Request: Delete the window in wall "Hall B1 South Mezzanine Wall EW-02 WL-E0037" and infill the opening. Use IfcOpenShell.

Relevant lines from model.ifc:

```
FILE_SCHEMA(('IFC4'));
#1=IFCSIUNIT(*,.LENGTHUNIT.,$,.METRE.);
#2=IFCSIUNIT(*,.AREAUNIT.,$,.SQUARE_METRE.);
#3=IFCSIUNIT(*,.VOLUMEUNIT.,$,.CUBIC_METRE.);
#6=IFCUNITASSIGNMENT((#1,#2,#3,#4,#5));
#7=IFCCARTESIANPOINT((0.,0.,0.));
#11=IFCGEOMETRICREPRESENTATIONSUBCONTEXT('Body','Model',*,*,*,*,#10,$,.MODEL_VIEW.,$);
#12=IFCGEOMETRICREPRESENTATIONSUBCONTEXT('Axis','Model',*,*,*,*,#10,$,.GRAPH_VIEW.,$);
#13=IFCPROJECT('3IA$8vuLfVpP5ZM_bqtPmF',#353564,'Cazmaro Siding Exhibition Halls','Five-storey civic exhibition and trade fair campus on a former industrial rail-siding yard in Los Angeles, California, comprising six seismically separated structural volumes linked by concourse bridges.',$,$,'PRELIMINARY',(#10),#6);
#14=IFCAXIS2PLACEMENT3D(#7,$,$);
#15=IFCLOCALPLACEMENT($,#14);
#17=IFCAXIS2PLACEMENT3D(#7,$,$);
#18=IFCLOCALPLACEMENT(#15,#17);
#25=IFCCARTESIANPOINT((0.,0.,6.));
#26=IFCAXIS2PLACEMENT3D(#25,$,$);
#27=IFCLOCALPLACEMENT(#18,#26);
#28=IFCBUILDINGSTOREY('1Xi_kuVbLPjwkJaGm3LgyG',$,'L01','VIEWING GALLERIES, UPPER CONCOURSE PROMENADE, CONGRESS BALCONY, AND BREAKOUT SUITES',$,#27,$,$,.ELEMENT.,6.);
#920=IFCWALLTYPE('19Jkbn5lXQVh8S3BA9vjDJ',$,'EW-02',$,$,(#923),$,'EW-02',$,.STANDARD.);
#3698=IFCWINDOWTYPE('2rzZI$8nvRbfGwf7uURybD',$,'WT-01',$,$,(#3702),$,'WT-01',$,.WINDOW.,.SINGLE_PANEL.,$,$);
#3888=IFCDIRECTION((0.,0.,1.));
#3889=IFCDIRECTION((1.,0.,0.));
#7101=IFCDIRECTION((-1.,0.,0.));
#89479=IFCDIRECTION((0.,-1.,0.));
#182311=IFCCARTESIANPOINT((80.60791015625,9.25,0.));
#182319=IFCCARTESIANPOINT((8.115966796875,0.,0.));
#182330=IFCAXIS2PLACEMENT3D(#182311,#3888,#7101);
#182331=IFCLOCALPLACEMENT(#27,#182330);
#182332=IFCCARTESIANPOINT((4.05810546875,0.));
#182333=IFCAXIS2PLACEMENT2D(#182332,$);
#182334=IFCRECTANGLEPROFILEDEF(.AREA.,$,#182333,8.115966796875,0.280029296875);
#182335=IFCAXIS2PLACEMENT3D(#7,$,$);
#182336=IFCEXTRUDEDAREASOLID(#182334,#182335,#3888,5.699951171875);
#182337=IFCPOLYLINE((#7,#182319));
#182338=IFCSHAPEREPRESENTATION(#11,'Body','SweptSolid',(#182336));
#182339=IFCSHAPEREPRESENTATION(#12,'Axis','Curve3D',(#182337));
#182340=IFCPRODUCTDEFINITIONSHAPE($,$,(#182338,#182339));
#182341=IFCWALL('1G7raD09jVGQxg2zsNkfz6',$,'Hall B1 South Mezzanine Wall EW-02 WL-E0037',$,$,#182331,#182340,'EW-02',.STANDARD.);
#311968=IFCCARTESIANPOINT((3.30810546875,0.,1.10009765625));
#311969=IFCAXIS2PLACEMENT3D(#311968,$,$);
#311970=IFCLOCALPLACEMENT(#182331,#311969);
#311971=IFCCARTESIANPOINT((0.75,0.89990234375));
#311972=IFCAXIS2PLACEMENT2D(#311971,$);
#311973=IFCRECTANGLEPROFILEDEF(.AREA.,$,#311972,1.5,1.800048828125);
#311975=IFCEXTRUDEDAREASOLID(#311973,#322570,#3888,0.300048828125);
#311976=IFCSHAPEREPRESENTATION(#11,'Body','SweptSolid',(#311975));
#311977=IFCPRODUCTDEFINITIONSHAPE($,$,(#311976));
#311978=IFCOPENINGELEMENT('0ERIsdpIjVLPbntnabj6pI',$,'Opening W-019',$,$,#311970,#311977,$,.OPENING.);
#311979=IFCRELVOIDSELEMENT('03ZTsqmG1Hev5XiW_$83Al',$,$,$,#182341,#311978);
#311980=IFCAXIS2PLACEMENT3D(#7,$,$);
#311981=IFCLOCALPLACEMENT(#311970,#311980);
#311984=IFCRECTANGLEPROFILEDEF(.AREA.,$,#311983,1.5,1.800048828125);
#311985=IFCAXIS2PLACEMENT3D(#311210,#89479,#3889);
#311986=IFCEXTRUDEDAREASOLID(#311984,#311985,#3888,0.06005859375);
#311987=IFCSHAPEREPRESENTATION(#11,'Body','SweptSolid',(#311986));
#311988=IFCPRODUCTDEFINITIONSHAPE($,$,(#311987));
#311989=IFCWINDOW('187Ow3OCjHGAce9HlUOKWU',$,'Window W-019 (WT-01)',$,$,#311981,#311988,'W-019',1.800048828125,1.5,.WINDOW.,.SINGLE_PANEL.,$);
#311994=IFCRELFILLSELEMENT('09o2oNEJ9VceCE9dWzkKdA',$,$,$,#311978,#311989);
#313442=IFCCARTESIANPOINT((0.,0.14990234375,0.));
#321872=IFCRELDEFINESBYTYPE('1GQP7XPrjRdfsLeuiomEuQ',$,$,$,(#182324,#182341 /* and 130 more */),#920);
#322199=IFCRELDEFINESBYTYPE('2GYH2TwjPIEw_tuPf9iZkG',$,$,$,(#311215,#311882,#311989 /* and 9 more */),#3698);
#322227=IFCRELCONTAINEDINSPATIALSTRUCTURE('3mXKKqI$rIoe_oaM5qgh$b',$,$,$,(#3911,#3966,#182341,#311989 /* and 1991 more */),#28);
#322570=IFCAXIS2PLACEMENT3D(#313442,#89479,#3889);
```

```python
import ifcopenshell
import ifcopenshell.api.feature
import ifcopenshell.api.root
import ifcopenshell.geom
import ifcopenshell.util.shape

model = ifcopenshell.open("model.ifc")
settings = ifcopenshell.geom.settings()


def volume(element):
    """Net volume in cubic metres, openings subtracted."""
    shape = ifcopenshell.geom.create_shape(settings, element)
    return ifcopenshell.util.shape.get_volume(shape.geometry)


window = model.by_id(311989)
opening = window.FillsVoids[0].RelatingOpeningElement
wall = opening.VoidsElements[0].RelatingBuildingElement
before = volume(wall)

ifcopenshell.api.root.remove_product(model, product=window)
ifcopenshell.api.feature.remove_feature(model, feature=opening)

after = volume(wall)

print(f"wall volume {before:.3f} -> {after:.3f} m3")

model.write("model_rev.ifc")
```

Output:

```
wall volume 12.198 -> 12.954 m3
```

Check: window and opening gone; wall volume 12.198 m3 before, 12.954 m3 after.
